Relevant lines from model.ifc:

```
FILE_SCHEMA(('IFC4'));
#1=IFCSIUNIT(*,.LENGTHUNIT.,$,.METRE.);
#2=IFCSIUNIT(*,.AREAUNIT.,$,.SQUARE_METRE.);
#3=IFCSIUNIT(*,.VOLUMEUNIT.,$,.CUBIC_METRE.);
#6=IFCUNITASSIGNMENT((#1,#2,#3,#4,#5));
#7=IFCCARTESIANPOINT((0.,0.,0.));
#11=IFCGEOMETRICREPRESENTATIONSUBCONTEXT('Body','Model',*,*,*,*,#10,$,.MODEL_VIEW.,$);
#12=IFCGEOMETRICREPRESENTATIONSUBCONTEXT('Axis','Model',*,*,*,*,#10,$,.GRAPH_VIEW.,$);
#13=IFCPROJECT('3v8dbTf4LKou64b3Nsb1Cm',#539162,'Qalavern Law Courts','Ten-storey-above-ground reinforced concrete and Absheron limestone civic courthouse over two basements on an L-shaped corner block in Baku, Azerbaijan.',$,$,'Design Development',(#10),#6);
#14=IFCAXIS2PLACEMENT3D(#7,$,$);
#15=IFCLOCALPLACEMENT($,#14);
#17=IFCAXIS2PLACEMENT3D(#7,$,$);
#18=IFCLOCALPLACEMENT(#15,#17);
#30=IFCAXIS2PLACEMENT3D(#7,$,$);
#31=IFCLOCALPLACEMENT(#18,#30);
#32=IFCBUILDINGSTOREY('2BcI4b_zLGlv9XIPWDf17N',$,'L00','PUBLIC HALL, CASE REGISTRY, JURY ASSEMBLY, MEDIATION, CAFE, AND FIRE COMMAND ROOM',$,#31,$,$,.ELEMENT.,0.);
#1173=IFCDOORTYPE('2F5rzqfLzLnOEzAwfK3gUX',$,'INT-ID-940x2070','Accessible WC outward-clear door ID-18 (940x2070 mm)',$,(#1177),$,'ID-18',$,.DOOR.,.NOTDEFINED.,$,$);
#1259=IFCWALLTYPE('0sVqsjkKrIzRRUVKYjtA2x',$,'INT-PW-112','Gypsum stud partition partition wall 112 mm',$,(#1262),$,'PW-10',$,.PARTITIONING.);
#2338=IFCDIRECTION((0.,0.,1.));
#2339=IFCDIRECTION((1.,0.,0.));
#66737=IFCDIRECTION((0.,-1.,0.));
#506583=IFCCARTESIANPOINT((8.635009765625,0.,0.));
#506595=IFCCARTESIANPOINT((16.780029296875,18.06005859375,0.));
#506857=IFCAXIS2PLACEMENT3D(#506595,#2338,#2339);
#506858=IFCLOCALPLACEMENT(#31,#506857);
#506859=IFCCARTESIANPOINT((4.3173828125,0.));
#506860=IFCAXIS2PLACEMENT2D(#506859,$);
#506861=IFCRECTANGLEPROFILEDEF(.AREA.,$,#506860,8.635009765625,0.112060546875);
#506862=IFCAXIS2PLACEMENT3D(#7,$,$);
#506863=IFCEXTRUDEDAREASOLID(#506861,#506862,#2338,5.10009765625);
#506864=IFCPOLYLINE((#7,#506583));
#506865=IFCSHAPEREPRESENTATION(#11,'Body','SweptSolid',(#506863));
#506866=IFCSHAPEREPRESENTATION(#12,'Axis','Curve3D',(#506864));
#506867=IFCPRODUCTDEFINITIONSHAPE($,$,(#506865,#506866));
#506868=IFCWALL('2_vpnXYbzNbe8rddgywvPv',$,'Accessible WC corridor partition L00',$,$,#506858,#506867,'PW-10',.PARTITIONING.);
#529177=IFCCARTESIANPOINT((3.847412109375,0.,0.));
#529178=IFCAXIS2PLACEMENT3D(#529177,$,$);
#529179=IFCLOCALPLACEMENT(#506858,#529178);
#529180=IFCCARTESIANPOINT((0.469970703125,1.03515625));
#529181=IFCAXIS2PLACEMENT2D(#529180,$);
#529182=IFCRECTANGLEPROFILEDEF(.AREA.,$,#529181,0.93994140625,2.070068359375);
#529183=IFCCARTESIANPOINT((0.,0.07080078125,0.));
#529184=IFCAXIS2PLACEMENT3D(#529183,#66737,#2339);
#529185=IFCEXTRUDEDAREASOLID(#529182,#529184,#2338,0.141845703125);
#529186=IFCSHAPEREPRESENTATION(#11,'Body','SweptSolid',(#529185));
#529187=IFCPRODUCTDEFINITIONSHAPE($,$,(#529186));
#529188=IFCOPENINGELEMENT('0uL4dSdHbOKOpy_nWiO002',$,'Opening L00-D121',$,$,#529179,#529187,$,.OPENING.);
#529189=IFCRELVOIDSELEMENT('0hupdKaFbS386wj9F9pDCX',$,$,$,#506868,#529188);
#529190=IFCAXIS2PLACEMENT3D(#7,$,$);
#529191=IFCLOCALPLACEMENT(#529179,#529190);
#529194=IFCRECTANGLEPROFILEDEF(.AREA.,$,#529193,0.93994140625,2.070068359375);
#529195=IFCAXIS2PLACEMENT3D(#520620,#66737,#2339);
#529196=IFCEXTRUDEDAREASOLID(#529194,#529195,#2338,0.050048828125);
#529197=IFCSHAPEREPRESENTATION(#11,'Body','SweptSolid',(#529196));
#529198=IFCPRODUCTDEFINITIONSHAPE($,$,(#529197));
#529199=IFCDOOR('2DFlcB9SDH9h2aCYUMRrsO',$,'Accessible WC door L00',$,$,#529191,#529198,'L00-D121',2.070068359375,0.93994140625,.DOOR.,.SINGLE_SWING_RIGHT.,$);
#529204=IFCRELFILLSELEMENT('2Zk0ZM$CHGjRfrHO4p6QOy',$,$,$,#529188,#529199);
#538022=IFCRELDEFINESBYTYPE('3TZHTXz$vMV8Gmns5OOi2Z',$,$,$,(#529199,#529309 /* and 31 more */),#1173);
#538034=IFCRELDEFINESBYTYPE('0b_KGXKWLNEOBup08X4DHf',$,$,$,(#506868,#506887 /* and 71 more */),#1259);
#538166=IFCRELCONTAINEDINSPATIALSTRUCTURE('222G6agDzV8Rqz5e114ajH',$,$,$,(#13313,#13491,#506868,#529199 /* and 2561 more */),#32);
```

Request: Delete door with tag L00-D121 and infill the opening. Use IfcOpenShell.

```python
import ifcopenshell
import ifcopenshell.api.feature
import ifcopenshell.api.root
import ifcopenshell.geom
import ifcopenshell.util.shape

model = ifcopenshell.open("model.ifc")
settings = ifcopenshell.geom.settings()


def volume(element):
    """Net volume in cubic metres, openings subtracted."""
    shape = ifcopenshell.geom.create_shape(settings, element)
    return ifcopenshell.util.shape.get_volume(shape.geometry)


door = model.by_id(529199)
opening = door.FillsVoids[0].RelatingOpeningElement
wall = opening.VoidsElements[0].RelatingBuildingElement
before = volume(wall)

ifcopenshell.api.root.remove_product(model, product=door)
ifcopenshell.api.feature.remove_feature(model, feature=opening)

after = volume(wall)

print(f"wall volume {before:.3f} -> {after:.3f} m3")

model.write("model_updated.ifc")
```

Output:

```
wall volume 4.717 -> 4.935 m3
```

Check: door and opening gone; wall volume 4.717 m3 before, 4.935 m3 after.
